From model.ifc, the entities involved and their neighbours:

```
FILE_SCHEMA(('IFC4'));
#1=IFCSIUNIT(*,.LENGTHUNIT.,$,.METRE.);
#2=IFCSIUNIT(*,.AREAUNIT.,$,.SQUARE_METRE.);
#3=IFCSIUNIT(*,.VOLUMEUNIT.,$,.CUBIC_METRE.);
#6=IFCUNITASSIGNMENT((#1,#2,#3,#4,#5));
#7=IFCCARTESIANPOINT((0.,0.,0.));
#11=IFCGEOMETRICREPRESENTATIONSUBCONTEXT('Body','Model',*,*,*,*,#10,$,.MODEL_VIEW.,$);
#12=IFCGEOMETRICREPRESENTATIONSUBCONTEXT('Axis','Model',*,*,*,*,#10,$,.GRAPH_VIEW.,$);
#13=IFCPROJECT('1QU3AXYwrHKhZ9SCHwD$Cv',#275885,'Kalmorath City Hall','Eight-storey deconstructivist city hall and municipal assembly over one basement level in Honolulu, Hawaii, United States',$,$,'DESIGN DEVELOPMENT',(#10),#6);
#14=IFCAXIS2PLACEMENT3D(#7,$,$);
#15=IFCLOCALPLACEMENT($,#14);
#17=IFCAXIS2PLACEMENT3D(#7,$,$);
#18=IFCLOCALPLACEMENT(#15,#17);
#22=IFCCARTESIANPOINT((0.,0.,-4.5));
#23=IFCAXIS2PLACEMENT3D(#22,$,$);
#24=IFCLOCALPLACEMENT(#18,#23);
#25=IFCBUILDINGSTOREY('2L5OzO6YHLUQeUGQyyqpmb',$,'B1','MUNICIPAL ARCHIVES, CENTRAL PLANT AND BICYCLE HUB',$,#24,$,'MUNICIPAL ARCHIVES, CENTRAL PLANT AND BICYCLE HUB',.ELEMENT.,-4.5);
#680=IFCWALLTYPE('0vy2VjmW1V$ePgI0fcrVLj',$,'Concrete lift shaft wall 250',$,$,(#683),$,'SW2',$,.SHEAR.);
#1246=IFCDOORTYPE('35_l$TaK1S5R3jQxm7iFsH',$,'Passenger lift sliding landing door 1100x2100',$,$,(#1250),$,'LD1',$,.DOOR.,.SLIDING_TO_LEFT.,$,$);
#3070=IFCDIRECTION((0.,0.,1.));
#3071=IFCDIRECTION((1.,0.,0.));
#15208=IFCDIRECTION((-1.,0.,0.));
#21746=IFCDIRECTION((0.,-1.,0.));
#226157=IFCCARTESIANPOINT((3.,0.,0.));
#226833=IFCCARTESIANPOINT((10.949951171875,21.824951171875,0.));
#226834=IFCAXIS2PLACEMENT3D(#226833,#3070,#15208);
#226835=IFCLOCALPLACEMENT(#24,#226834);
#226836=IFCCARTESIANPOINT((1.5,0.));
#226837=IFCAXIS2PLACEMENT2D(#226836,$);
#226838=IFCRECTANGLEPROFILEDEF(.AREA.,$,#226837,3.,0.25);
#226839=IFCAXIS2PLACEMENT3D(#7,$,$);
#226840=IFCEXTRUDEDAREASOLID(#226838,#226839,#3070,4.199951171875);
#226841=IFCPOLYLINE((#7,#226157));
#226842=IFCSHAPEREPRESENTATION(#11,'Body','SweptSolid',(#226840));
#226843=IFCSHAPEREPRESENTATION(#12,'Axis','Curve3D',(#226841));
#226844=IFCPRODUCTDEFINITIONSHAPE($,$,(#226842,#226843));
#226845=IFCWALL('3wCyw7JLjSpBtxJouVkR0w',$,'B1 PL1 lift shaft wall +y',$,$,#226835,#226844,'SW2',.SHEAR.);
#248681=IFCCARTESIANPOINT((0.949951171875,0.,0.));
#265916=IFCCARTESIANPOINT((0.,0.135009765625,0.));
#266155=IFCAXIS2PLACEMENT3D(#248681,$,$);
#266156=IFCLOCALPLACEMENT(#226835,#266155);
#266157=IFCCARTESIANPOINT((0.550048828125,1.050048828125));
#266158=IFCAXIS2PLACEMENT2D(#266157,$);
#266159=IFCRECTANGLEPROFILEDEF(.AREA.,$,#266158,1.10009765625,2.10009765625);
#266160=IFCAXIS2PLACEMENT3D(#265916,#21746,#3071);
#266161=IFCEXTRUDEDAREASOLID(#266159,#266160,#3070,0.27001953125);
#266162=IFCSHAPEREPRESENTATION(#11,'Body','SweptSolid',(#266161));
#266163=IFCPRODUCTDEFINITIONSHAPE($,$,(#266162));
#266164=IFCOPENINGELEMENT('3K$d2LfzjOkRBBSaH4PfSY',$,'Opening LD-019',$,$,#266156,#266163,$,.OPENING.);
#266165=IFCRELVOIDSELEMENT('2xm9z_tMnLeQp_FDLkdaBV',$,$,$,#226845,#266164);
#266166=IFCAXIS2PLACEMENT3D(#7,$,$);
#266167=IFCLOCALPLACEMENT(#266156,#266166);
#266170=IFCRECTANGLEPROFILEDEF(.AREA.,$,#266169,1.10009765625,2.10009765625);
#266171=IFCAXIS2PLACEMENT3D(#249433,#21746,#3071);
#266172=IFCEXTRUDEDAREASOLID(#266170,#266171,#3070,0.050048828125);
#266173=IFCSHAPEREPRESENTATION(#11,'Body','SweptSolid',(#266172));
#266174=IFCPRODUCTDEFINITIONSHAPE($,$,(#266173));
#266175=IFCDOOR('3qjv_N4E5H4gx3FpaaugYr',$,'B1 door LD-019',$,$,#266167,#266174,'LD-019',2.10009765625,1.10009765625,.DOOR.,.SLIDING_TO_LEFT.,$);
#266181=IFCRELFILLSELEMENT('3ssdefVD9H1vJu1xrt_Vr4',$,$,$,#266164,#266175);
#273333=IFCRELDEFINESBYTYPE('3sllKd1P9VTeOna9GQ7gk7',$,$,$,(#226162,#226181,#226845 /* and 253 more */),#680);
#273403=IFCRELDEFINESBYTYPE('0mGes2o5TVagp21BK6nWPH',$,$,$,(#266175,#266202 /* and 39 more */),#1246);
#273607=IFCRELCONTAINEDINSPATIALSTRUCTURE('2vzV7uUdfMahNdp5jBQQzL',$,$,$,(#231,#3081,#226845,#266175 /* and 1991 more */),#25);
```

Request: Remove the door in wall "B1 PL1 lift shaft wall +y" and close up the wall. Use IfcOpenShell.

```python
import ifcopenshell
import ifcopenshell.api.feature
import ifcopenshell.api.root
import ifcopenshell.geom
import ifcopenshell.util.shape

model = ifcopenshell.open("model.ifc")
settings = ifcopenshell.geom.settings()


def volume(element):
    """Net volume in cubic metres, openings subtracted."""
    shape = ifcopenshell.geom.create_shape(settings, element)
    return ifcopenshell.util.shape.get_volume(shape.geometry)


door = model.by_id(266175)
opening = door.FillsVoids[0].RelatingOpeningElement
wall = opening.VoidsElements[0].RelatingBuildingElement
before = volume(wall)

ifcopenshell.api.root.remove_product(model, product=door)
ifcopenshell.api.feature.remove_feature(model, feature=opening)

after = volume(wall)

print(f"wall volume {before:.3f} -> {after:.3f} m3")

model.write("model_updated.ifc")
```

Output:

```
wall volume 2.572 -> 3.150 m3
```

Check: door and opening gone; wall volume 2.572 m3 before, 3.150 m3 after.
